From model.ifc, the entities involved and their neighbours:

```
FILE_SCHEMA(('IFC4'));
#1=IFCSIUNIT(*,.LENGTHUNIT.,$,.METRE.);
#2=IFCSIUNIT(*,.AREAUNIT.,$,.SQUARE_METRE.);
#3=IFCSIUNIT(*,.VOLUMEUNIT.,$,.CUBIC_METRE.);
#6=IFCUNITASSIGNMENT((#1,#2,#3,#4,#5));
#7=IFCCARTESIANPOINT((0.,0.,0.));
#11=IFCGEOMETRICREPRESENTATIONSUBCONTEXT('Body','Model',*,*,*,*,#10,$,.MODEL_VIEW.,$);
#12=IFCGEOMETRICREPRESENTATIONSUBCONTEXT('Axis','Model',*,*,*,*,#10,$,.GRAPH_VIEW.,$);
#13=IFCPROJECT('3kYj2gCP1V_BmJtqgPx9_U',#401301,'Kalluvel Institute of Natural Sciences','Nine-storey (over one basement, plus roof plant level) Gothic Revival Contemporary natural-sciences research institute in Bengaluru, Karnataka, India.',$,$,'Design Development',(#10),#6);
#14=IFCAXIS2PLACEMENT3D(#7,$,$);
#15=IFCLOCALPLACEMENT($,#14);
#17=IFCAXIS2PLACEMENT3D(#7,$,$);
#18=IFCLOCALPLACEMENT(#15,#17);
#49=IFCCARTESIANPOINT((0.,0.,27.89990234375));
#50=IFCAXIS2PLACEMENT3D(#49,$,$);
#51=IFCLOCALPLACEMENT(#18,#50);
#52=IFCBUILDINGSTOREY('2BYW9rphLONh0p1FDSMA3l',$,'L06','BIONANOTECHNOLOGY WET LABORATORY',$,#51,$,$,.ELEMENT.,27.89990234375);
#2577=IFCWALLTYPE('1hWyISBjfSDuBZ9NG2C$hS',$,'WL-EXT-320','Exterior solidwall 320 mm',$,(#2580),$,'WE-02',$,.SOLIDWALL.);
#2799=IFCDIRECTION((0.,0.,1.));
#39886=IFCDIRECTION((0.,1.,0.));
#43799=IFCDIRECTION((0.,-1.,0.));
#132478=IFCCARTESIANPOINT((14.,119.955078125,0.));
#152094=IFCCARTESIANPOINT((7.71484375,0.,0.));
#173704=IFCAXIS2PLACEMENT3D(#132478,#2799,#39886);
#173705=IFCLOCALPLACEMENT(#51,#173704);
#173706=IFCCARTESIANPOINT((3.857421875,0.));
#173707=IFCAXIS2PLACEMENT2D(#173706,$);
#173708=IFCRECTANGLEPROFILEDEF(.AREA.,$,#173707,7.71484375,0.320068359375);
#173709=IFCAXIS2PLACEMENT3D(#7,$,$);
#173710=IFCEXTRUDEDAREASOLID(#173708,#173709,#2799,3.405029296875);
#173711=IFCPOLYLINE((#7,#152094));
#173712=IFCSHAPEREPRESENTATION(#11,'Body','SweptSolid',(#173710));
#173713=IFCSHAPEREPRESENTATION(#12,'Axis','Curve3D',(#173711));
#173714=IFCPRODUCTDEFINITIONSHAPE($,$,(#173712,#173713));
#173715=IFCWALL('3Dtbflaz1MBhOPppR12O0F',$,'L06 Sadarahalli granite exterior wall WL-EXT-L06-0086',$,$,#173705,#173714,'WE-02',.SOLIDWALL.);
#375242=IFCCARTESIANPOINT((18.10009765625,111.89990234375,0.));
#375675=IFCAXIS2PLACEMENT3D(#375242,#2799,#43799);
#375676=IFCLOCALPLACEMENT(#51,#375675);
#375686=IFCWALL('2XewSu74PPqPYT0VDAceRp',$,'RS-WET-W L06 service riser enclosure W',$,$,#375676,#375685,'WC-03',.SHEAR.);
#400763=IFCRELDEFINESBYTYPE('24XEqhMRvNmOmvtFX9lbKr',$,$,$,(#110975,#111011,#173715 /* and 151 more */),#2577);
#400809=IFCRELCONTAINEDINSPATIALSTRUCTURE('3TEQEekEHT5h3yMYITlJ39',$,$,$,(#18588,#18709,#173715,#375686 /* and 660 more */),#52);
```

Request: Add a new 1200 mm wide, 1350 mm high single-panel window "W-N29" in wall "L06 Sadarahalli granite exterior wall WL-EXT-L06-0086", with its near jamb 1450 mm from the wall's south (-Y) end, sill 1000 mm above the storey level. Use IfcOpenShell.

```python
import numpy as np
import ifcopenshell
import ifcopenshell.api.feature
import ifcopenshell.api.geometry
import ifcopenshell.api.root
import ifcopenshell.api.spatial
import ifcopenshell.geom
import ifcopenshell.util.element
import ifcopenshell.util.placement
import ifcopenshell.util.representation
import ifcopenshell.util.shape
import ifcopenshell.util.unit

model = ifcopenshell.open("model.ifc")
unit_scale = ifcopenshell.util.unit.calculate_unit_scale(model)
settings = ifcopenshell.geom.settings()


def volume(element):
    """Net volume in cubic metres, openings subtracted."""
    shape = ifcopenshell.geom.create_shape(settings, element)
    return ifcopenshell.util.shape.get_volume(shape.geometry)


wall = model.by_guid("3Dtbflaz1MBhOPppR12O0F")
storey = ifcopenshell.util.element.get_container(wall, ifc_class="IfcBuildingStorey")
context = ifcopenshell.util.representation.get_context(model, "Model", "Body", "MODEL_VIEW")
before = volume(wall)

width, height, from_end, sill = 1.2, 1.35, 1.45, 1  # metres

# The wall runs along its own X axis, and the end named is its -X end.
wall_shape = ifcopenshell.geom.create_shape(settings, wall)
x, y, z = ifcopenshell.util.shape.get_vertices(wall_shape.geometry).T
start = x.min() + from_end
face, thickness = float(y.min()), float(y.max() - y.min())
wall_matrix = ifcopenshell.util.placement.get_local_placement(wall.ObjectPlacement)
level = ifcopenshell.util.placement.get_local_placement(storey.ObjectPlacement)[2, 3]


def in_wall(x, y):
    """Placement at x, y metres in the wall's axes, at sill height."""
    matrix = wall_matrix.copy()
    matrix[:, 3] = wall_matrix @ np.array([x / unit_scale, y / unit_scale, 0.0, 1.0])
    matrix[2, 3] = level + sill / unit_scale
    return matrix


# Opening: a box that overshoots both wall faces by 50 mm.
opening = ifcopenshell.api.root.create_entity(model, ifc_class="IfcOpeningElement", predefined_type="OPENING")
box = ifcopenshell.api.geometry.add_wall_representation(
    model, context=context, length=width, height=height, thickness=thickness + 0.1
)
ifcopenshell.api.geometry.assign_representation(model, product=opening, representation=box)
ifcopenshell.api.geometry.edit_object_placement(model, product=opening, matrix=in_wall(start, face - 0.05), is_si=False)
ifcopenshell.api.feature.add_feature(model, feature=opening, element=wall)

window = ifcopenshell.api.root.create_entity(model, ifc_class="IfcWindow", name="W-N29", predefined_type="WINDOW")
window.OverallWidth, window.OverallHeight = width / unit_scale, height / unit_scale
window.PartitioningType = "SINGLE_PANEL"
body = ifcopenshell.api.geometry.add_window_representation(
    model,
    context=context,
    overall_width=window.OverallWidth,
    overall_height=window.OverallHeight,
    partition_type="SINGLE_PANEL",
)
ifcopenshell.api.geometry.assign_representation(model, product=window, representation=body)
ifcopenshell.api.spatial.assign_container(model, products=[window], relating_structure=storey)
ifcopenshell.api.feature.add_filling(model, opening=opening, element=window)

# Centre the window in the wall's thickness.
ifcopenshell.api.geometry.edit_object_placement(model, product=window, matrix=in_wall(start, face), is_si=False)
window_shape = ifcopenshell.geom.create_shape(settings, window)
depth = ifcopenshell.util.shape.get_vertices(window_shape.geometry)[:, 1]
offset = face + thickness / 2 - (depth.min() + depth.max()) / 2
ifcopenshell.api.geometry.edit_object_placement(model, product=window, matrix=in_wall(start, offset), is_si=False)

after = volume(wall)

print(f"wall volume {before:.3f} -> {after:.3f} m3")

model.write("model_updated.ifc")
```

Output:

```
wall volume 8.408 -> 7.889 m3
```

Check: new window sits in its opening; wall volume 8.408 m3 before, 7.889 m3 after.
